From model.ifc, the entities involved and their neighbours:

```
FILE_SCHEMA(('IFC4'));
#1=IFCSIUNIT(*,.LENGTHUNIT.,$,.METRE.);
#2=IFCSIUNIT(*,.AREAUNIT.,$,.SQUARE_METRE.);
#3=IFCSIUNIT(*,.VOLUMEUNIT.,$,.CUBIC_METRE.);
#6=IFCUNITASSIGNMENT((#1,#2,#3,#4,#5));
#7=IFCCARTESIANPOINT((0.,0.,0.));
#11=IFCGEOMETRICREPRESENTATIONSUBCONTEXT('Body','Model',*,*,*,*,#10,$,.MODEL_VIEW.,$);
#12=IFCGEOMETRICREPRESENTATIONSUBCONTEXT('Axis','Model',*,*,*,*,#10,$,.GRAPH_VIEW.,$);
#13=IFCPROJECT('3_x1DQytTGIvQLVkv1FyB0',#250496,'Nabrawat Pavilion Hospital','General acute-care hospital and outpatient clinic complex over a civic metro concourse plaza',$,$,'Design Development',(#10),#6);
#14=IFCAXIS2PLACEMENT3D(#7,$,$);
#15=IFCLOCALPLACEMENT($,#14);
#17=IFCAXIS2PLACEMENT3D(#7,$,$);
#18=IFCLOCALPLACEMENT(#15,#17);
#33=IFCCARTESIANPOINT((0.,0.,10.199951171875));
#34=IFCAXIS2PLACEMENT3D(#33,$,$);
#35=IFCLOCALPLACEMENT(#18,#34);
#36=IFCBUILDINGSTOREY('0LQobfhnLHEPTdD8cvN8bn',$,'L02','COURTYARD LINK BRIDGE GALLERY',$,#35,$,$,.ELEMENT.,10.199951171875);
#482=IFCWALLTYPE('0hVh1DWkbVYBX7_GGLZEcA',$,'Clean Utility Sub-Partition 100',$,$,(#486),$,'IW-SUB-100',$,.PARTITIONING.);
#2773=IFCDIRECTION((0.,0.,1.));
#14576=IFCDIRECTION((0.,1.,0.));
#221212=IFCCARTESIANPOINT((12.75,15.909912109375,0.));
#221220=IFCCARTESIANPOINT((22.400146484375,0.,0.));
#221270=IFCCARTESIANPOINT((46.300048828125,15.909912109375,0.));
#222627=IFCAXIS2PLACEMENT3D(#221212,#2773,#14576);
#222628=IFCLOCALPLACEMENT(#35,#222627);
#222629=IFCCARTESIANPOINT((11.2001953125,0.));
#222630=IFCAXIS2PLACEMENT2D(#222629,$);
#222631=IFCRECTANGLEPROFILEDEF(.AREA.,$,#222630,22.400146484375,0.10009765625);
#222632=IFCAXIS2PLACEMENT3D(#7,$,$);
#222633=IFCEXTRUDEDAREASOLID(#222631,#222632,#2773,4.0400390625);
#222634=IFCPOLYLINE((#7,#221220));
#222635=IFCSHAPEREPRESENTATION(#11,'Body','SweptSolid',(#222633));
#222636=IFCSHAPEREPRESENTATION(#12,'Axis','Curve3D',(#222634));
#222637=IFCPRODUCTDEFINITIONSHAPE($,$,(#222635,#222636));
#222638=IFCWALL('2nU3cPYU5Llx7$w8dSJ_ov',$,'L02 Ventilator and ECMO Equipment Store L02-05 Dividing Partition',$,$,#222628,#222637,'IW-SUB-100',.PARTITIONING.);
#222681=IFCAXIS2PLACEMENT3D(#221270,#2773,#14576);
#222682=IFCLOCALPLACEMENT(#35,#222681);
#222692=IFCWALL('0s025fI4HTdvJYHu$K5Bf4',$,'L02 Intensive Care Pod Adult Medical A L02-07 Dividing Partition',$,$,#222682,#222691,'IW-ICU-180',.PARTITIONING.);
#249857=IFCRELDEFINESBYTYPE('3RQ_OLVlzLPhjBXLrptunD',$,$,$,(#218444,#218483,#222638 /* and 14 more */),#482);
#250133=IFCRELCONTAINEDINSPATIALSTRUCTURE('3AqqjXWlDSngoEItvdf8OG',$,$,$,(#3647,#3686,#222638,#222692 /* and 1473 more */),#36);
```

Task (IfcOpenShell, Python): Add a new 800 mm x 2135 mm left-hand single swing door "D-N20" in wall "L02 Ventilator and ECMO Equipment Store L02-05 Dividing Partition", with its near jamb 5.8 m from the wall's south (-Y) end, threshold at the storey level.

```python
import numpy as np
import ifcopenshell
import ifcopenshell.api.feature
import ifcopenshell.api.geometry
import ifcopenshell.api.root
import ifcopenshell.api.spatial
import ifcopenshell.geom
import ifcopenshell.util.element
import ifcopenshell.util.placement
import ifcopenshell.util.representation
import ifcopenshell.util.shape
import ifcopenshell.util.unit

model = ifcopenshell.open("model.ifc")
unit_scale = ifcopenshell.util.unit.calculate_unit_scale(model)
settings = ifcopenshell.geom.settings()


def volume(element):
    """Net volume in cubic metres, openings subtracted."""
    shape = ifcopenshell.geom.create_shape(settings, element)
    return ifcopenshell.util.shape.get_volume(shape.geometry)


wall = model.by_id(222638)
storey = ifcopenshell.util.element.get_container(wall, ifc_class="IfcBuildingStorey")
context = ifcopenshell.util.representation.get_context(model, "Model", "Body", "MODEL_VIEW")
before = volume(wall)

width, height, from_end, sill = 0.8, 2.135, 5.8, 0.0  # metres

# The wall runs along its own X axis, and the end named is its -X end.
wall_shape = ifcopenshell.geom.create_shape(settings, wall)
x, y, z = ifcopenshell.util.shape.get_vertices(wall_shape.geometry).T
start = x.min() + from_end
face, thickness = float(y.min()), float(y.max() - y.min())
wall_matrix = ifcopenshell.util.placement.get_local_placement(wall.ObjectPlacement)
level = ifcopenshell.util.placement.get_local_placement(storey.ObjectPlacement)[2, 3]


def in_wall(x, y):
    """Placement at x, y metres in the wall's axes, at sill height."""
    matrix = wall_matrix.copy()
    matrix[:, 3] = wall_matrix @ np.array([x / unit_scale, y / unit_scale, 0.0, 1.0])
    matrix[2, 3] = level + sill / unit_scale
    return matrix


# Opening: a box that overshoots both wall faces by 50 mm.
opening = ifcopenshell.api.root.create_entity(model, ifc_class="IfcOpeningElement", predefined_type="OPENING")
box = ifcopenshell.api.geometry.add_wall_representation(
    model, context=context, length=width, height=height, thickness=thickness + 0.1
)
ifcopenshell.api.geometry.assign_representation(model, product=opening, representation=box)
ifcopenshell.api.geometry.edit_object_placement(model, product=opening, matrix=in_wall(start, face - 0.05), is_si=False)
ifcopenshell.api.feature.add_feature(model, feature=opening, element=wall)

door = ifcopenshell.api.root.create_entity(model, ifc_class="IfcDoor", name="D-N20", predefined_type="DOOR")
door.OverallWidth, door.OverallHeight = width / unit_scale, height / unit_scale
door.OperationType = "SINGLE_SWING_LEFT"
body = ifcopenshell.api.geometry.add_door_representation(
    model,
    context=context,
    overall_width=door.OverallWidth,
    overall_height=door.OverallHeight,
    operation_type="SINGLE_SWING_LEFT",
    lining_properties={"LiningDepth": thickness / unit_scale, "ThresholdDepth": thickness / unit_scale},
)
ifcopenshell.api.geometry.assign_representation(model, product=door, representation=body)
ifcopenshell.api.spatial.assign_container(model, products=[door], relating_structure=storey)
ifcopenshell.api.feature.add_filling(model, opening=opening, element=door)

# The lining spans the wall, so the door starts at the wall face.
ifcopenshell.api.geometry.edit_object_placement(model, product=door, matrix=in_wall(start, face), is_si=False)

after = volume(wall)

print(f"wall volume {before:.3f} -> {after:.3f} m3")

model.write("model_v2.ifc")
```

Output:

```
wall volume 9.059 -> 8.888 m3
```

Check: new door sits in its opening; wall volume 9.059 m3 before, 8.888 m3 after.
